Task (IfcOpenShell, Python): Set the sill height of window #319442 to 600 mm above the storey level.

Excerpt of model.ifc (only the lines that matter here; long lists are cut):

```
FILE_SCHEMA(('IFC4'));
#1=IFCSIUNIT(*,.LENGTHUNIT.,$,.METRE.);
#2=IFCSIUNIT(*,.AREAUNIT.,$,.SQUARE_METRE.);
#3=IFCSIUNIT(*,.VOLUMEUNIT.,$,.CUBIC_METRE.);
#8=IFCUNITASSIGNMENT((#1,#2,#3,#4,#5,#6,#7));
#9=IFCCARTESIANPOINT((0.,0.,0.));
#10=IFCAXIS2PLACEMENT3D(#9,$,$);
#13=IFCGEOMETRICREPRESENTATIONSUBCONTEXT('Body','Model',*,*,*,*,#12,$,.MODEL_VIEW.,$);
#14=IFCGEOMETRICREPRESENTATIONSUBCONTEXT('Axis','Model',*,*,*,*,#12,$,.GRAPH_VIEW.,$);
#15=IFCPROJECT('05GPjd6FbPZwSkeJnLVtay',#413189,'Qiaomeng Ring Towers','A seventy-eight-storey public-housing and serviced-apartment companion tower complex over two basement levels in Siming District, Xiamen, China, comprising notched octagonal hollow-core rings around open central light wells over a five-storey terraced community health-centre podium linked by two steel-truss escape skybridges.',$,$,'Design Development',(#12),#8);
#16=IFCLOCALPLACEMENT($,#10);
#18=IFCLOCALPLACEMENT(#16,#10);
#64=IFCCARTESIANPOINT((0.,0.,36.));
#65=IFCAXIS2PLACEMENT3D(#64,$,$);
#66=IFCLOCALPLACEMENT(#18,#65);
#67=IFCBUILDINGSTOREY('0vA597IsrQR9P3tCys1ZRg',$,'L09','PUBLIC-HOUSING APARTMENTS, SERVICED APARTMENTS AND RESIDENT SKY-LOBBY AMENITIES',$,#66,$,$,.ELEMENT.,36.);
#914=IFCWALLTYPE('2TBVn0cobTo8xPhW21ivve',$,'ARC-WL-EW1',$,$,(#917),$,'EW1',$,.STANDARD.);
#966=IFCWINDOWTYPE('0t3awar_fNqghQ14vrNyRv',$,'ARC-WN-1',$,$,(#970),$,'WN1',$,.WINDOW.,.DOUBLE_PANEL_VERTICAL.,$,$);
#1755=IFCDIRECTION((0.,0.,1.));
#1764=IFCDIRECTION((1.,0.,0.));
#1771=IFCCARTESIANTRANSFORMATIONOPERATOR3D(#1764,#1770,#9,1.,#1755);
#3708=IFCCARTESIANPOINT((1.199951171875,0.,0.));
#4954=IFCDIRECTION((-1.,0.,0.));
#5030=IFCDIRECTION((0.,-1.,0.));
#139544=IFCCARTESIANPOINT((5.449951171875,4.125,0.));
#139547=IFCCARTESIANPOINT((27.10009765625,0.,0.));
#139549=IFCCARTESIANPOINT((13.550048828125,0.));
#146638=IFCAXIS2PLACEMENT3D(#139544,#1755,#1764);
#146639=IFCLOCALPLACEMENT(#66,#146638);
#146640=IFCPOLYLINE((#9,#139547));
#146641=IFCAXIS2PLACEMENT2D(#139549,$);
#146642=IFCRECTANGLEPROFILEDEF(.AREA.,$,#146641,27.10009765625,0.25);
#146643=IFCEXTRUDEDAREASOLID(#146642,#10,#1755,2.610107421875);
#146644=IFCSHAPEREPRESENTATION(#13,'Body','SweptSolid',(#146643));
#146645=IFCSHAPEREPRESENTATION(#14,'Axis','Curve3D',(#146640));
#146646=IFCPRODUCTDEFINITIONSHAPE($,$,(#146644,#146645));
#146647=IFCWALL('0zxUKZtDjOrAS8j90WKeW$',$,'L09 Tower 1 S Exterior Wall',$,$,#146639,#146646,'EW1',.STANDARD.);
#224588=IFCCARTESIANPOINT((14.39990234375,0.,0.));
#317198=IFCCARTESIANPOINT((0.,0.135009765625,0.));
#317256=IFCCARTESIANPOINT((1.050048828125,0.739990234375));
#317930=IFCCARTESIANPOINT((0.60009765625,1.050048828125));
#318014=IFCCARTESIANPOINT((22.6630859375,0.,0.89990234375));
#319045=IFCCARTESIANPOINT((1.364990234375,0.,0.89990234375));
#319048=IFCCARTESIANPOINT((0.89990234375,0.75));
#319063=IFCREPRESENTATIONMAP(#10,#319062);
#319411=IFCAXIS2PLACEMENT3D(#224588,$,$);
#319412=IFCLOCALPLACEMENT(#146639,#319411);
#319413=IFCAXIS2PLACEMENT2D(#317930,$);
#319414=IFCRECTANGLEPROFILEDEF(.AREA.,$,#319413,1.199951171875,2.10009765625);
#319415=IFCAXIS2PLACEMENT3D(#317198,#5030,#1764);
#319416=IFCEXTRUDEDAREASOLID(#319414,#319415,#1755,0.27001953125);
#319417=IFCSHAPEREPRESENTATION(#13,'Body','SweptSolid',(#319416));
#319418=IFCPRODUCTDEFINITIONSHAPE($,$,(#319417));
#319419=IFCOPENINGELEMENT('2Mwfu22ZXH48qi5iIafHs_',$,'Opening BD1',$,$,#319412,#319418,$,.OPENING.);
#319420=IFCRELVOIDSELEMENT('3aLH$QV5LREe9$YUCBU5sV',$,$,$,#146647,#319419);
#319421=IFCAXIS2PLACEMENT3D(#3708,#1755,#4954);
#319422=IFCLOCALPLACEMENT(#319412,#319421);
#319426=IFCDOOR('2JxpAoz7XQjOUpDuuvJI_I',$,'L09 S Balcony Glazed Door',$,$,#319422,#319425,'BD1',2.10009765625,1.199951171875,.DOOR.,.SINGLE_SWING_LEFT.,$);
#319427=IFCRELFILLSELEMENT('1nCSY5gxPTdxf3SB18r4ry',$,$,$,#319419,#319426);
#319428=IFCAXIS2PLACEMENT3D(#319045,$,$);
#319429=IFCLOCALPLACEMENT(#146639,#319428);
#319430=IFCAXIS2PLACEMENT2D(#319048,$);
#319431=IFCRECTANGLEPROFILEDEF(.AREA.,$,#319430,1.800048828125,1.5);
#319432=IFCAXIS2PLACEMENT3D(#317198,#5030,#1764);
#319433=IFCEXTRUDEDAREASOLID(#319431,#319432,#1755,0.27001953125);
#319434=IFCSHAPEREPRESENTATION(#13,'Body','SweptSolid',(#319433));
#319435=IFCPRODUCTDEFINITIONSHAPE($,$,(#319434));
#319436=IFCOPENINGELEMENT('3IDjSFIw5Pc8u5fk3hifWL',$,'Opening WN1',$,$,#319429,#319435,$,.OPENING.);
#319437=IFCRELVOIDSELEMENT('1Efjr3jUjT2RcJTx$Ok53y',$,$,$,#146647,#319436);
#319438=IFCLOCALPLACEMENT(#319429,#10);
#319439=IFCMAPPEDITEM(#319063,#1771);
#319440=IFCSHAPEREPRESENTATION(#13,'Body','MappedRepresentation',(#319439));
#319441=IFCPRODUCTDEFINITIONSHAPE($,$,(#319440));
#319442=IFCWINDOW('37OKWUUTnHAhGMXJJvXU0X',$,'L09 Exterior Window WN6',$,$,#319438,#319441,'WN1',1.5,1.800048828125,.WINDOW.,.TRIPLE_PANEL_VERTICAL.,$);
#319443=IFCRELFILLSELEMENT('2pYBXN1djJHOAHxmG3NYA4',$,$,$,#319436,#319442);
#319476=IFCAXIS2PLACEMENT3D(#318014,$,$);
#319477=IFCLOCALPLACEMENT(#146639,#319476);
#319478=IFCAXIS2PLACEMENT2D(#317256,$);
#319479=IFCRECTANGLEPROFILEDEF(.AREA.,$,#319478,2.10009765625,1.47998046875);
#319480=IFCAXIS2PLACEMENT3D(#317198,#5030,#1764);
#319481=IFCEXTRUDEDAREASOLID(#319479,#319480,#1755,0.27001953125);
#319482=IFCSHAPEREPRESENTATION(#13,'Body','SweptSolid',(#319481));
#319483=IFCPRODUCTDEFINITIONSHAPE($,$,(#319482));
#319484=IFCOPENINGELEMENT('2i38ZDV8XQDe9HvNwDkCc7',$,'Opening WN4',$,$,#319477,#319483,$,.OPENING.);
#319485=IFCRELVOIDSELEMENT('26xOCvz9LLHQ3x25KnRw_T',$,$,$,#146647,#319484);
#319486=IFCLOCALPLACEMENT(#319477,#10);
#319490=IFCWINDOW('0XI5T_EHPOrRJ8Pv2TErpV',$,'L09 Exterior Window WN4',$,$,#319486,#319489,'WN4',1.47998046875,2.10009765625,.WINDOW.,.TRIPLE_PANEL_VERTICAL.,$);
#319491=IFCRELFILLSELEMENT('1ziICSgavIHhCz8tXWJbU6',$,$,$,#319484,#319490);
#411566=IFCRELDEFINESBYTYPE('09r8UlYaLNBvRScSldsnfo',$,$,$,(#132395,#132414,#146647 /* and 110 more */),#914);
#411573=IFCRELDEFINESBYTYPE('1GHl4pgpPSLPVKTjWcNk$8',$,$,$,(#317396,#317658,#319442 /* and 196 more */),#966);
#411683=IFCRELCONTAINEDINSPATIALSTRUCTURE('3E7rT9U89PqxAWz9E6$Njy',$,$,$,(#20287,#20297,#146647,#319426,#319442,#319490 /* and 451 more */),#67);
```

```python
import numpy as np
import ifcopenshell
import ifcopenshell.api.geometry
import ifcopenshell.geom
import ifcopenshell.util.element
import ifcopenshell.util.placement
import ifcopenshell.util.shape
import ifcopenshell.util.unit

model = ifcopenshell.open("model.ifc")
unit_scale = ifcopenshell.util.unit.calculate_unit_scale(model)

window = model.by_guid("37OKWUUTnHAhGMXJJvXU0X")
opening = window.FillsVoids[0].RelatingOpeningElement
storey = ifcopenshell.util.element.get_container(window, ifc_class="IfcBuildingStorey")
level = ifcopenshell.util.placement.get_local_placement(storey.ObjectPlacement)[2, 3]

# The opening's origin need not be at the sill, so measure its lowest point.
shape = ifcopenshell.geom.create_shape(ifcopenshell.geom.settings(), opening)
bottom = ifcopenshell.util.shape.get_shape_bottom_elevation(shape, shape.geometry) / unit_scale
dz = level + 0.6 / unit_scale - bottom

shift = np.array([0.0, 0.0, dz])
# The window is placed relative to its opening, so it follows when the opening moves.
matrix = ifcopenshell.util.placement.get_local_placement(opening.ObjectPlacement)
matrix[:3, 3] += shift
ifcopenshell.api.geometry.edit_object_placement(
    model, product=opening, matrix=matrix, is_si=False, should_transform_children=True
)

print(f"moved by {dz * unit_scale:+.3f} m")

model.write("model-out.ifc")
```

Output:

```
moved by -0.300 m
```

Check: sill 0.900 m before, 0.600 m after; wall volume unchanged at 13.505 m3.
